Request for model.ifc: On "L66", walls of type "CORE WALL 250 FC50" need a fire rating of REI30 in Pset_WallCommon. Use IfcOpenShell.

First a look at what the model holds.

```python
import ifcopenshell
import ifcopenshell.util.element

model = ifcopenshell.open("model.ifc")
print(model.schema)
storey = next(s for s in model.by_type("IfcBuildingStorey") if s.Name == "L66")
walls = [e for e in ifcopenshell.util.element.get_decomposition(storey) if e.is_a("IfcWall")]
seen = {}
for e in walls:
    element_type = ifcopenshell.util.element.get_type(e)
    key = (element_type.Name if element_type != e and element_type else None, ifcopenshell.util.element.get_pset(e, "Pset_WallCommon", "FireRating"))
    seen[key] = seen.get(key, 0) + 1
for (name, value), count in sorted(seen.items(), key=str):
    print(count, "x", name, "|", value)
```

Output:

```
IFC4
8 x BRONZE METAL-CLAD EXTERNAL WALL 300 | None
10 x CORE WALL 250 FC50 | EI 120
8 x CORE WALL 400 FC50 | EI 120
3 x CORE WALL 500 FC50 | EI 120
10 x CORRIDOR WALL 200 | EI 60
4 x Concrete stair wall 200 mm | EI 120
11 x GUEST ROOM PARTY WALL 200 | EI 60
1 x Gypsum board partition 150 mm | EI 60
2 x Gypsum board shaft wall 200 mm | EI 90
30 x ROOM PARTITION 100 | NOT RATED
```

```python
import ifcopenshell
import ifcopenshell.api.pset
import ifcopenshell.util.element

model = ifcopenshell.open("model.ifc")

storey = next(s for s in model.by_type("IfcBuildingStorey") if s.Name == "L66")
walls = [e for e in ifcopenshell.util.element.get_decomposition(storey) if e.is_a("IfcWall")]

count = 0
for e in walls:
    element_type = ifcopenshell.util.element.get_type(e)
    if element_type in (None, e) or element_type.Name != "CORE WALL 250 FC50":
        continue
    found = ifcopenshell.util.element.get_pset(e, "Pset_WallCommon", should_inherit=False)
    if found:
        pset = model.by_id(found["id"])
        if len(ifcopenshell.util.element.get_elements_by_pset(pset)) > 1:
            pset = ifcopenshell.api.pset.unshare_pset(model, products=[e], pset=pset)[0]
    else:
        pset = ifcopenshell.api.pset.add_pset(model, product=e, name="Pset_WallCommon")
    ifcopenshell.api.pset.edit_pset(model, pset=pset, properties={"FireRating": "REI30"})
    count += 1

print(count, "walls updated")

model.write("model_rev.ifc")
```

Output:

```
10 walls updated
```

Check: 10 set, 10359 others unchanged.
